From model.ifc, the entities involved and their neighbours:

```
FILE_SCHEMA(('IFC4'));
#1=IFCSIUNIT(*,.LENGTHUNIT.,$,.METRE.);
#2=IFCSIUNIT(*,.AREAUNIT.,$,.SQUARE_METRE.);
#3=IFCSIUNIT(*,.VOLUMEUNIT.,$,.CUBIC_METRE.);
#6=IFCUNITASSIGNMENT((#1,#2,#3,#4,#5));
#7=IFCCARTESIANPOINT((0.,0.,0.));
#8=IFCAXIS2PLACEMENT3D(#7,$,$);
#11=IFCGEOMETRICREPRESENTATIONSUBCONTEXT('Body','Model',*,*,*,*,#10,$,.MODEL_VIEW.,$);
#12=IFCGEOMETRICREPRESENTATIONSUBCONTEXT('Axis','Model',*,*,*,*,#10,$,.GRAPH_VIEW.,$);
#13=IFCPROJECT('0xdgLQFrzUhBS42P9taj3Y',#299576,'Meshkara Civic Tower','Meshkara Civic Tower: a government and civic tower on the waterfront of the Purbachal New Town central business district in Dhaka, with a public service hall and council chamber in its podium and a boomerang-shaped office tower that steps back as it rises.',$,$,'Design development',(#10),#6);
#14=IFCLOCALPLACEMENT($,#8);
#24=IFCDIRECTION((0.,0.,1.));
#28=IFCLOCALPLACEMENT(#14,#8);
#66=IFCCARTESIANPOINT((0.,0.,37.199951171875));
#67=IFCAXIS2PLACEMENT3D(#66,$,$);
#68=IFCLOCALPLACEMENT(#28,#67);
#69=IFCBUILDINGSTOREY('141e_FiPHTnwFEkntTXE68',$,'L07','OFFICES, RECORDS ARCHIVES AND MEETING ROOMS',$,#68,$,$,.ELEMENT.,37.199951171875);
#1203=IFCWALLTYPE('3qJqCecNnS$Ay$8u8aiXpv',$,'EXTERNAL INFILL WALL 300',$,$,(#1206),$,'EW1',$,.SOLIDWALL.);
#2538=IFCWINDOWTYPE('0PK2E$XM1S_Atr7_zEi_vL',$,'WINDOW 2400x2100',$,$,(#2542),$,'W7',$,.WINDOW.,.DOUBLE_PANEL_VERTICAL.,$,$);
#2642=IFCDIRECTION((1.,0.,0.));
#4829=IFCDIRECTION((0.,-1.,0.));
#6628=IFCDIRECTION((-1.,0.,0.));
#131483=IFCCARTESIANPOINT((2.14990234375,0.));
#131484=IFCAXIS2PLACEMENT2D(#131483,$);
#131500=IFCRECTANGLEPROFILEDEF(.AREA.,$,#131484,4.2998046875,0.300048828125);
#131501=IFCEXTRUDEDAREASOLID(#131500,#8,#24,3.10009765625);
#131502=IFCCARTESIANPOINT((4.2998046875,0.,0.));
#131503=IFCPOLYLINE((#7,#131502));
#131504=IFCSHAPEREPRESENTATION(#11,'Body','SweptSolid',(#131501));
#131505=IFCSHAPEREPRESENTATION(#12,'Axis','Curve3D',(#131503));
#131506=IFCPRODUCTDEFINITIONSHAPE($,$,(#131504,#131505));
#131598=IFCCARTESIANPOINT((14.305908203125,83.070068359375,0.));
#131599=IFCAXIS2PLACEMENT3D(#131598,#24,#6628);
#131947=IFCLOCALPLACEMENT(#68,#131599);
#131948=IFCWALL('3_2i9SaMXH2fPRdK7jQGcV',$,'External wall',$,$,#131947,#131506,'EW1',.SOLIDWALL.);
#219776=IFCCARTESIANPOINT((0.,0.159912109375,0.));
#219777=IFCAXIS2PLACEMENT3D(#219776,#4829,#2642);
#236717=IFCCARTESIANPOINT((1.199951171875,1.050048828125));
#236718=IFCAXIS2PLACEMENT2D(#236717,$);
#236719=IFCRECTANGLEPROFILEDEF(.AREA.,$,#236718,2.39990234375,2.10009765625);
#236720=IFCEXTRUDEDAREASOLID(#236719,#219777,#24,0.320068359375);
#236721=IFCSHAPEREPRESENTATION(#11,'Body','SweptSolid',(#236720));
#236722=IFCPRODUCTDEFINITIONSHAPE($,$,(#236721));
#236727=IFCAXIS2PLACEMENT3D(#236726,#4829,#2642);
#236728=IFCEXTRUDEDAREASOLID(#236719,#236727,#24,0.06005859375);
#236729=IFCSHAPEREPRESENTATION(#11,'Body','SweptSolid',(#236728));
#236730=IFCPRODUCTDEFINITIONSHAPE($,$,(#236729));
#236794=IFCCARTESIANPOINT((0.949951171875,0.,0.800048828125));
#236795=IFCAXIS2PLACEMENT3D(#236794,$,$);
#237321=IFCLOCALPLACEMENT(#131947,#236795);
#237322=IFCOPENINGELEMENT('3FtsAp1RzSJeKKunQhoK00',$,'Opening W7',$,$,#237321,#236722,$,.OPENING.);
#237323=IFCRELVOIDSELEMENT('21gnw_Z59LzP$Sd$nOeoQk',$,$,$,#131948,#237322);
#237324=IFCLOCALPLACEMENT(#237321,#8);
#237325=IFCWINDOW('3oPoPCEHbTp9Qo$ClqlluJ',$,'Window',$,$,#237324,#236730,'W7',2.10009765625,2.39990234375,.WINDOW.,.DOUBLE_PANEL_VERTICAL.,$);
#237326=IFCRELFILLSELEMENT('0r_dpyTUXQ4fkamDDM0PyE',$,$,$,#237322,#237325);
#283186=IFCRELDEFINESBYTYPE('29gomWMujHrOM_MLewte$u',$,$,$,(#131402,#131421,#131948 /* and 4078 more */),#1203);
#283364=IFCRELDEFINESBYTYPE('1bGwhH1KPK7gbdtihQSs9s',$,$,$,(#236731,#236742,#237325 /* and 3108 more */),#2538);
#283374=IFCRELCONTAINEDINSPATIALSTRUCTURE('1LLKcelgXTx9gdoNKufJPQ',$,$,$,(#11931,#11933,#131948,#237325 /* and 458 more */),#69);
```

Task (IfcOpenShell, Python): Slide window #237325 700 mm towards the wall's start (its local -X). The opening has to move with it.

```python
import ifcopenshell
import ifcopenshell.api.geometry
import ifcopenshell.util.placement
import ifcopenshell.util.unit

model = ifcopenshell.open("model.ifc")
unit_scale = ifcopenshell.util.unit.calculate_unit_scale(model)

window = model.by_guid("3oPoPCEHbTp9Qo$ClqlluJ")
opening = window.FillsVoids[0].RelatingOpeningElement
wall = opening.VoidsElements[0].RelatingBuildingElement

wall_matrix = ifcopenshell.util.placement.get_local_placement(wall.ObjectPlacement)
shift = wall_matrix[:3, 0] * -0.7 / unit_scale
before = ifcopenshell.util.placement.get_local_placement(window.ObjectPlacement)[:3, 3].copy()

# The window is placed relative to its opening, so it follows when the opening moves.
matrix = ifcopenshell.util.placement.get_local_placement(opening.ObjectPlacement)
matrix[:3, 3] += shift
ifcopenshell.api.geometry.edit_object_placement(
    model, product=opening, matrix=matrix, is_si=False, should_transform_children=True
)

after = ifcopenshell.util.placement.get_local_placement(window.ObjectPlacement)[:3, 3]
print("window moved by", (after - before).round(3) + 0.0)

model.write("model_v2.ifc")
```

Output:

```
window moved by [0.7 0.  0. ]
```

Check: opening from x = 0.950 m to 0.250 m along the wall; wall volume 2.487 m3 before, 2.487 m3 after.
